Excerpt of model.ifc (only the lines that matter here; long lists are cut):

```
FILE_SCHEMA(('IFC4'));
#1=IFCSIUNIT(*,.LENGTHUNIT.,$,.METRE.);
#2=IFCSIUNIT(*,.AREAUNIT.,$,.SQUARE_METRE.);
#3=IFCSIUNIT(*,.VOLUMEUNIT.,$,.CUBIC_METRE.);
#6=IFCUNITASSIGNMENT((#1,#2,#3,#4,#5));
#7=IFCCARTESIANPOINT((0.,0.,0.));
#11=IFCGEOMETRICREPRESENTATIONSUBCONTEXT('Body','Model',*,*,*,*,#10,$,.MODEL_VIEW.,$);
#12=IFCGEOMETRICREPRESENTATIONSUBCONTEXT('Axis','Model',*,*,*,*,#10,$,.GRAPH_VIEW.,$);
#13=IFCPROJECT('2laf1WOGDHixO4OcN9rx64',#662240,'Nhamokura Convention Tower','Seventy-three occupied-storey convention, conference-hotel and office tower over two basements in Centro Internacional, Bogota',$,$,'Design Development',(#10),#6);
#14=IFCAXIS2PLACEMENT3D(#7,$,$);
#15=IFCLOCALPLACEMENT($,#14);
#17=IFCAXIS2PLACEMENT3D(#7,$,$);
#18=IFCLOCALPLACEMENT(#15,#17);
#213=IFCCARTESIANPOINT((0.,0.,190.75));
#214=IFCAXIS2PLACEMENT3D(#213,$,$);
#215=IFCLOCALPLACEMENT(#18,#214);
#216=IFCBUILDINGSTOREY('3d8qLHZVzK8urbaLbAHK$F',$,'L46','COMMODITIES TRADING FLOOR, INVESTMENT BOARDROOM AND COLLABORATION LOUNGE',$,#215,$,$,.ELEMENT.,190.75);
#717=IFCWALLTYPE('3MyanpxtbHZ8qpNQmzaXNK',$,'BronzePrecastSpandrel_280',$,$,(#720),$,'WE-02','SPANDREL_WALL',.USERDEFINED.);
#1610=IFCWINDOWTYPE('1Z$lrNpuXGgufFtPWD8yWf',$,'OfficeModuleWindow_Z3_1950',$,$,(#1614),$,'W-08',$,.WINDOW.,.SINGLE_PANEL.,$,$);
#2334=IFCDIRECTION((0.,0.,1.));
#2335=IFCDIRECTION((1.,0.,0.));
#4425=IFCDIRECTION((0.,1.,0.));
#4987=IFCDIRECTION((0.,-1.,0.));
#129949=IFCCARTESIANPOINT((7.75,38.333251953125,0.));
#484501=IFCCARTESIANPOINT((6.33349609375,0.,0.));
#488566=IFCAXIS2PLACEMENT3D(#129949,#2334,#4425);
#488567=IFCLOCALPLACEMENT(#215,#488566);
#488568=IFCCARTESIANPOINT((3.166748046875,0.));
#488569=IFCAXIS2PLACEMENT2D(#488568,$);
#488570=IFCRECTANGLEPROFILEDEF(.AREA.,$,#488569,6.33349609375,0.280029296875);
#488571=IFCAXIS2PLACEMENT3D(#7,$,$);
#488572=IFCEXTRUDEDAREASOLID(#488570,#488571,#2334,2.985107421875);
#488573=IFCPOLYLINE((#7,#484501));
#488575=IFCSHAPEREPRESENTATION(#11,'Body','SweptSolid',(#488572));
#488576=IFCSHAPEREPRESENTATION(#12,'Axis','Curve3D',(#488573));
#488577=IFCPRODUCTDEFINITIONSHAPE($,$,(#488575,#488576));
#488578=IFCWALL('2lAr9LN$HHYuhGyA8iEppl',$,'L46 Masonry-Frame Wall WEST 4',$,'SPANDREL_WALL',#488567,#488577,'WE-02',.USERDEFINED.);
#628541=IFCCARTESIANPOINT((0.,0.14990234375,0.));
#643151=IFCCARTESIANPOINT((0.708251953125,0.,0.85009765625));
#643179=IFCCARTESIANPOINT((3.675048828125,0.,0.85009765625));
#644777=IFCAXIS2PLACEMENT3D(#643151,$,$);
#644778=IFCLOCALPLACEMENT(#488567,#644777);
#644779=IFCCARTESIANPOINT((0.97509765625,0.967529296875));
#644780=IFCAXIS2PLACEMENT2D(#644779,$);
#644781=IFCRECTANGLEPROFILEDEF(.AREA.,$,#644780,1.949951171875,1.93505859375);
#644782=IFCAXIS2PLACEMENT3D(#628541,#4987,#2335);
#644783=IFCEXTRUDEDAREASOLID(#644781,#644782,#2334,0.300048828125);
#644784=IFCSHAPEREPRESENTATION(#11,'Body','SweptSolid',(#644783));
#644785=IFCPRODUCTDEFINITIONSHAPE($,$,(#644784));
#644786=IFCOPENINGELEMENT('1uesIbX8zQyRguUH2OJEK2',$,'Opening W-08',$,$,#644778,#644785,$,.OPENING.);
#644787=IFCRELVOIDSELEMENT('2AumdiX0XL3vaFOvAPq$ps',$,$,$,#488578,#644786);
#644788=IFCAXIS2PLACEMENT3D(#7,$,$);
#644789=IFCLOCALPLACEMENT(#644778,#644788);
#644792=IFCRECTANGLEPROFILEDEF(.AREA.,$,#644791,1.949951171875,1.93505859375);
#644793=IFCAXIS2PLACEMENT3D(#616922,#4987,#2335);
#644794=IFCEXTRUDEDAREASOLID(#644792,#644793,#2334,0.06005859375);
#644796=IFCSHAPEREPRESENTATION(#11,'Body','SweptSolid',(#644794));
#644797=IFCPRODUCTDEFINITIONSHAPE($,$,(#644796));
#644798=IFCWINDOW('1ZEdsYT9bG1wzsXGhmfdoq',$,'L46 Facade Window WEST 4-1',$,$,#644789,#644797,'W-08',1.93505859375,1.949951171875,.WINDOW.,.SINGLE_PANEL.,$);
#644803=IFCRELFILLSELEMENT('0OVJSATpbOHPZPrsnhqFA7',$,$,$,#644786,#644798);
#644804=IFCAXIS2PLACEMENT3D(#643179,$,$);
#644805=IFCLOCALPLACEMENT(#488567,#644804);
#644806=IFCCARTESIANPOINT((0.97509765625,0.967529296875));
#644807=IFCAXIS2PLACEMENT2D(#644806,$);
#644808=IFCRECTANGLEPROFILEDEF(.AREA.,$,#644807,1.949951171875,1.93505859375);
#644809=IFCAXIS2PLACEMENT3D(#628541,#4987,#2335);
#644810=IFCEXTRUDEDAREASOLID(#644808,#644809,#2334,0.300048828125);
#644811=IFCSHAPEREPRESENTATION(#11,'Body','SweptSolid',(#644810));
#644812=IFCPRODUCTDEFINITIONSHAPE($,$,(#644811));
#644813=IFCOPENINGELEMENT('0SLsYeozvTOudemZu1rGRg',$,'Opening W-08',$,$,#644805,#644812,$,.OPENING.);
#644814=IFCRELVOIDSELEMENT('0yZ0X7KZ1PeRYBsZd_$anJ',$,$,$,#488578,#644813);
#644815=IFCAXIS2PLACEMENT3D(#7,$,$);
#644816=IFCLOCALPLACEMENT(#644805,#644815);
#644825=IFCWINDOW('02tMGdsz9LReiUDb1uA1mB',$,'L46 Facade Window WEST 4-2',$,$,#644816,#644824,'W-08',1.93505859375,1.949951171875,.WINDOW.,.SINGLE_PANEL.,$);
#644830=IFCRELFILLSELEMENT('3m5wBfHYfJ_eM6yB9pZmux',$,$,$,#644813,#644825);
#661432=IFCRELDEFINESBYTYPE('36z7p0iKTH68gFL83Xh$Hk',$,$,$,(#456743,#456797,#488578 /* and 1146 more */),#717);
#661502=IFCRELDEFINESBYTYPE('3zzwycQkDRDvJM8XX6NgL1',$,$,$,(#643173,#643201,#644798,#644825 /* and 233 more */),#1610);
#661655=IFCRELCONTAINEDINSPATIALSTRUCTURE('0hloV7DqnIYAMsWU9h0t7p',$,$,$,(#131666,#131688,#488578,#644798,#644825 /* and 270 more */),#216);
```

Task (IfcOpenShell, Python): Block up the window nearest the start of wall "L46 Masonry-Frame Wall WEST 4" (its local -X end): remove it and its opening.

```python
import ifcopenshell
import ifcopenshell.api.feature
import ifcopenshell.api.root
import ifcopenshell.geom
import ifcopenshell.util.shape

model = ifcopenshell.open("model.ifc")
settings = ifcopenshell.geom.settings()


def volume(element):
    """Net volume in cubic metres, openings subtracted."""
    shape = ifcopenshell.geom.create_shape(settings, element)
    return ifcopenshell.util.shape.get_volume(shape.geometry)


window = model.by_guid("1ZEdsYT9bG1wzsXGhmfdoq")
opening = window.FillsVoids[0].RelatingOpeningElement
wall = opening.VoidsElements[0].RelatingBuildingElement
before = volume(wall)

ifcopenshell.api.root.remove_product(model, product=window)
ifcopenshell.api.feature.remove_feature(model, feature=opening)

after = volume(wall)

print(f"wall volume {before:.3f} -> {after:.3f} m3")

model.write("model_rev.ifc")
```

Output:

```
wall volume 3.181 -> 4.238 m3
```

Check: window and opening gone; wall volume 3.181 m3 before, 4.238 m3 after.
